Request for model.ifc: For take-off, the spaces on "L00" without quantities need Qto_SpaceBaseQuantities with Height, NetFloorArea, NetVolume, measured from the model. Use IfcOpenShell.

First a look at what the model holds.

```python
import ifcopenshell
import ifcopenshell.util.element
import ifcopenshell.util.unit

model = ifcopenshell.open("model.ifc")
print(model.schema)
for unit_type in ("LENGTHUNIT", "AREAUNIT", "VOLUMEUNIT"):
    print(unit_type, ifcopenshell.util.unit.calculate_unit_scale(model, unit_type))
storey = next(s for s in model.by_type("IfcBuildingStorey") if s.Name == "L00")
spaces = [e for e in ifcopenshell.util.element.get_decomposition(storey) if e.is_a("IfcSpace")]
for e in sorted(spaces, key=lambda e: e.id()):
    print(e.id(), e.is_a(), e.Name, list(ifcopenshell.util.element.get_psets(e, qtos_only=True)), sep=" | ")
```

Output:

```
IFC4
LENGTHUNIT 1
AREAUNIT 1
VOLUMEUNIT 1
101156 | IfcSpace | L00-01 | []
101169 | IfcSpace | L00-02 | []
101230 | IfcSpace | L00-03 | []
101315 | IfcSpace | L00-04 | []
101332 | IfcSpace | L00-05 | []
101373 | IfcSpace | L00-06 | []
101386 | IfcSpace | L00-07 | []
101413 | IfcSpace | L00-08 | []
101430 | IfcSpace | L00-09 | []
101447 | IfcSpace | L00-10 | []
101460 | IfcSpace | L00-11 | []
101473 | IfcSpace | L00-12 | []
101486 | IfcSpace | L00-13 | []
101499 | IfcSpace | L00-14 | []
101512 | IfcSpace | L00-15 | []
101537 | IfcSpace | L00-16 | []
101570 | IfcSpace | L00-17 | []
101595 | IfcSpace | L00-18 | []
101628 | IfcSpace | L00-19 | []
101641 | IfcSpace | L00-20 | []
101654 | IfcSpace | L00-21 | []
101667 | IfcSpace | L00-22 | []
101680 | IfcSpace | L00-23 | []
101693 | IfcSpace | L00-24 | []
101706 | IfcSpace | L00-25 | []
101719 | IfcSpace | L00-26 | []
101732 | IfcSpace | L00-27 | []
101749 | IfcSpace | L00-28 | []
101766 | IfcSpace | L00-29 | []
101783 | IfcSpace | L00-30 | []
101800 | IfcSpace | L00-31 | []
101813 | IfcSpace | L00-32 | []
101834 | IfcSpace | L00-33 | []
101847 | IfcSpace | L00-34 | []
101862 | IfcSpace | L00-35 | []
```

```python
import ifcopenshell
import ifcopenshell.api.pset
import ifcopenshell.geom
import ifcopenshell.util.element
import ifcopenshell.util.shape
import ifcopenshell.util.unit

model = ifcopenshell.open("model.ifc")
unit_scale = ifcopenshell.util.unit.calculate_unit_scale(model)
area_scale = ifcopenshell.util.unit.calculate_unit_scale(model, "AREAUNIT")
volume_scale = ifcopenshell.util.unit.calculate_unit_scale(model, "VOLUMEUNIT")
settings = ifcopenshell.geom.settings()

storey = next(s for s in model.by_type("IfcBuildingStorey") if s.Name == "L00")
spaces = [e for e in ifcopenshell.util.element.get_decomposition(storey) if e.is_a("IfcSpace")]

for e in sorted(spaces, key=lambda e: e.id()):
    if ifcopenshell.util.element.get_psets(e, qtos_only=True, should_inherit=False):
        continue
    # Geometry comes back in metres, in the element's own axes.
    shape = ifcopenshell.geom.create_shape(settings, e)
    values = {
        "Height": ifcopenshell.util.shape.get_z(shape.geometry) / unit_scale,
        "NetFloorArea": ifcopenshell.util.shape.get_footprint_area(shape.geometry) / area_scale,
        "NetVolume": ifcopenshell.util.shape.get_volume(shape.geometry) / volume_scale,
    }
    qto = ifcopenshell.api.pset.add_qto(model, product=e, name="Qto_SpaceBaseQuantities")
    ifcopenshell.api.pset.edit_qto(model, qto=qto, properties=values)
    print(e.id(), {k: round(v, 3) for k, v in values.items()})

model.write("model_rev.ifc")
```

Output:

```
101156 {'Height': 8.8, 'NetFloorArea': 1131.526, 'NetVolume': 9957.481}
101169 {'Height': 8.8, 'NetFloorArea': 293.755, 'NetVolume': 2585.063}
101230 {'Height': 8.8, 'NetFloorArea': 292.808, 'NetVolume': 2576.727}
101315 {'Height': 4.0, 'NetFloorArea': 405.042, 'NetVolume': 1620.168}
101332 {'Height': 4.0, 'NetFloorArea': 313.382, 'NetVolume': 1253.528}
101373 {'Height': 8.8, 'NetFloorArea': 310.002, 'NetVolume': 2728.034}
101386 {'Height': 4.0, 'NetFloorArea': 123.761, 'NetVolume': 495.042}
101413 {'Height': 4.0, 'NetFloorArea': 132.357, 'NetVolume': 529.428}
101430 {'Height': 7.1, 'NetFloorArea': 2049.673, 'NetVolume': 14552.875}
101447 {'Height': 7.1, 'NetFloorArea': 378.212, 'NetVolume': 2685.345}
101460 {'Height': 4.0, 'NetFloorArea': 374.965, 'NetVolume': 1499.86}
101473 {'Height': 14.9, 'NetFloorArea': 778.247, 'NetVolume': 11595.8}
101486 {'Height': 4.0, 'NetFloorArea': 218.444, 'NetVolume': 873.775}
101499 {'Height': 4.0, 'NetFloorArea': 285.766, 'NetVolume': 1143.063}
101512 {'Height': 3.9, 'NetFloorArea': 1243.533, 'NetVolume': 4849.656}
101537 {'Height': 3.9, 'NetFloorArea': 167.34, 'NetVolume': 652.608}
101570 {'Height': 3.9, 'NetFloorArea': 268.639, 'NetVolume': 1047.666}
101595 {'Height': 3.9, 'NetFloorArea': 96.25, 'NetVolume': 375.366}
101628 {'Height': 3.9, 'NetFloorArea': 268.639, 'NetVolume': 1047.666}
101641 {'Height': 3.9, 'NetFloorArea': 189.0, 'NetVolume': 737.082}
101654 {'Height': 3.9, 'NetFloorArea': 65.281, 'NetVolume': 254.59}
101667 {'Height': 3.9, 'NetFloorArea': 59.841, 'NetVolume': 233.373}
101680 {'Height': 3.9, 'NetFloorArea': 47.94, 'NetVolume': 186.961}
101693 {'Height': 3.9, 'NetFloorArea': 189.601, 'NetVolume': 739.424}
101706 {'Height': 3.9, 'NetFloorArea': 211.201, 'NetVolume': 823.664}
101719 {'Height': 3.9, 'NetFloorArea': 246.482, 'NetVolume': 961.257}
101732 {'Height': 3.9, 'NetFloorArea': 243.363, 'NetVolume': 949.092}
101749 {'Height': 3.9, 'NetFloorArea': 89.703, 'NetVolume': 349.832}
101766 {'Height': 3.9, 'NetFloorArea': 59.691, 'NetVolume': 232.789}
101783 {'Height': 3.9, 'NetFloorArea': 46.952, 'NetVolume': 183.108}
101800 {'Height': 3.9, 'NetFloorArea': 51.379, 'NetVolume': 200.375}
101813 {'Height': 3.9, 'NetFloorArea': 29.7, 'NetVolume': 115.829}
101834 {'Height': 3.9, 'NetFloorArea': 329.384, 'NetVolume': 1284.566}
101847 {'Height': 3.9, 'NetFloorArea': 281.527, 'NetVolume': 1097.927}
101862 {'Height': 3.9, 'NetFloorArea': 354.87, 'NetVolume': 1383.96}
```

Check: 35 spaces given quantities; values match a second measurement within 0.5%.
